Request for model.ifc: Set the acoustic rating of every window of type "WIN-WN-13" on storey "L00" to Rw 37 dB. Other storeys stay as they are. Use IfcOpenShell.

First a look at what the model holds.

```python
import ifcopenshell
import ifcopenshell.util.element

model = ifcopenshell.open("model.ifc")
print(model.schema)
storey = next(s for s in model.by_type("IfcBuildingStorey") if s.Name == "L00")
windows = [e for e in ifcopenshell.util.element.get_decomposition(storey) if e.is_a("IfcWindow")]
seen = {}
for e in windows:
    element_type = ifcopenshell.util.element.get_type(e)
    key = (element_type.Name if element_type != e and element_type else None, ifcopenshell.util.element.get_pset(e, "Pset_WindowCommon", "AcousticRating"))
    seen[key] = seen.get(key, 0) + 1
for (name, value), count in sorted(seen.items(), key=str):
    print(count, "x", name, "|", value)
```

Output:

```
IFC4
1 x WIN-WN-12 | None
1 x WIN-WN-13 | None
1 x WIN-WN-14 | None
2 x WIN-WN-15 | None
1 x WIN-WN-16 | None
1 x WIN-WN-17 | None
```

```python
import ifcopenshell
import ifcopenshell.api.pset
import ifcopenshell.util.element

model = ifcopenshell.open("model.ifc")

storey = next(s for s in model.by_type("IfcBuildingStorey") if s.Name == "L00")
windows = [e for e in ifcopenshell.util.element.get_decomposition(storey) if e.is_a("IfcWindow")]

count = 0
for e in windows:
    element_type = ifcopenshell.util.element.get_type(e)
    if element_type in (None, e) or element_type.Name != "WIN-WN-13":
        continue
    # add_pset returns the element's existing set when there is one.
    pset = ifcopenshell.api.pset.add_pset(model, product=e, name="Pset_WindowCommon")
    ifcopenshell.api.pset.edit_pset(model, pset=pset, properties={"AcousticRating": "Rw 37 dB"})
    count += 1

print(count, "windows updated")

model.write("model_edited.ifc")
```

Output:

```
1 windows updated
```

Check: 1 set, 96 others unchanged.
